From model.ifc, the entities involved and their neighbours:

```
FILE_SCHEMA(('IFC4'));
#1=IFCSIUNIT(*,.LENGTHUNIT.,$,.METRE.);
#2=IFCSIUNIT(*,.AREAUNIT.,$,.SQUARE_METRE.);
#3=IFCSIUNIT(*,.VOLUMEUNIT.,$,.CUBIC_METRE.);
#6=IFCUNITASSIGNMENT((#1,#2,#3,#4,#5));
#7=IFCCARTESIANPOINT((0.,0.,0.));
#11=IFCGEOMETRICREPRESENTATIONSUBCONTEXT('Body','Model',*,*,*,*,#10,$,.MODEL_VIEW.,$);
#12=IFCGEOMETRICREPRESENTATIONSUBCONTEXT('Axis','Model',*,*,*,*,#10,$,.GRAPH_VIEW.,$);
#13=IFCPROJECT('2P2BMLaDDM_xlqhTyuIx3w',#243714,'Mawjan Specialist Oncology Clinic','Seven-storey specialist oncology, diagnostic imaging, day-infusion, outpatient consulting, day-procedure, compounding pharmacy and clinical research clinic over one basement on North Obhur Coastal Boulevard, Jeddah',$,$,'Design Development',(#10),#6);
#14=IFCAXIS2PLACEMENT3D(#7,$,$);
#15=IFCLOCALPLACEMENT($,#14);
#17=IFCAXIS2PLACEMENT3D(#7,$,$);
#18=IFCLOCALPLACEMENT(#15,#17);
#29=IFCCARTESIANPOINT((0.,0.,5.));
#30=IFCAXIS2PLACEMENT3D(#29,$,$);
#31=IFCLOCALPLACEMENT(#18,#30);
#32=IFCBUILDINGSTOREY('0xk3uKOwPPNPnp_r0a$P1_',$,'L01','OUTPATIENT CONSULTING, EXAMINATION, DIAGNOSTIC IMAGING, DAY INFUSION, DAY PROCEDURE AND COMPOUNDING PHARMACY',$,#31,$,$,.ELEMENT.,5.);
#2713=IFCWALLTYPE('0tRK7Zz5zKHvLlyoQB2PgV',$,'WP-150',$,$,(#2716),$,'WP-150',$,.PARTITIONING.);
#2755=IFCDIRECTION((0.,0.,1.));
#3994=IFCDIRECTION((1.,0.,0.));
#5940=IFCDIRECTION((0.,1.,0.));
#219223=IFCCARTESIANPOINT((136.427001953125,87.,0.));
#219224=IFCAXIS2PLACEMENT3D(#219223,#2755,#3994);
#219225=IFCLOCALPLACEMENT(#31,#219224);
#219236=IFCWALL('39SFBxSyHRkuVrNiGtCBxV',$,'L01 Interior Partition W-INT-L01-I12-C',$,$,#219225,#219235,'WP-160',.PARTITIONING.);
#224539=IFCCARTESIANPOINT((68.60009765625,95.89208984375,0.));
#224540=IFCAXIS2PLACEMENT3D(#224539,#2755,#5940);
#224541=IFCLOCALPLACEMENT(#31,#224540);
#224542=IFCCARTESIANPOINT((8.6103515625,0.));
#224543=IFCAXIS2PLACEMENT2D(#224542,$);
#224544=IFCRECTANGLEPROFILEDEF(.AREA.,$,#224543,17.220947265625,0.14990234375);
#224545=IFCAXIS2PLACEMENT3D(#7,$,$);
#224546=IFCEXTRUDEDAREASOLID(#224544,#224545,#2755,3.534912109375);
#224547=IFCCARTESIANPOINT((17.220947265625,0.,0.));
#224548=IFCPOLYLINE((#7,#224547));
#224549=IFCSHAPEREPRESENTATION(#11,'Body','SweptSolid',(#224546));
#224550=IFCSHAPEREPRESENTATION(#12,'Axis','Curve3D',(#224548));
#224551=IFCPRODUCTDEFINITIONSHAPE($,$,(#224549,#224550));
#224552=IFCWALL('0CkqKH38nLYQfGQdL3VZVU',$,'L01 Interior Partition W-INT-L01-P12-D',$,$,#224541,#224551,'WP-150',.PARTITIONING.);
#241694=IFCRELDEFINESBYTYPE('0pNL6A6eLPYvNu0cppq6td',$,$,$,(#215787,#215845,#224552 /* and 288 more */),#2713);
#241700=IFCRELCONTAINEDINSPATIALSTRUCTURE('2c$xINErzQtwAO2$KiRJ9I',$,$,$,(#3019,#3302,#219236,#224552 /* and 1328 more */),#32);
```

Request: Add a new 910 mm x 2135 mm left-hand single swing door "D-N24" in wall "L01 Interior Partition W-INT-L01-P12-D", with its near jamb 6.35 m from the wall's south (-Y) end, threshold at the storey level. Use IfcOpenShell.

```python
import numpy as np
import ifcopenshell
import ifcopenshell.api.feature
import ifcopenshell.api.geometry
import ifcopenshell.api.root
import ifcopenshell.api.spatial
import ifcopenshell.geom
import ifcopenshell.util.element
import ifcopenshell.util.placement
import ifcopenshell.util.representation
import ifcopenshell.util.shape
import ifcopenshell.util.unit

model = ifcopenshell.open("model.ifc")
unit_scale = ifcopenshell.util.unit.calculate_unit_scale(model)
settings = ifcopenshell.geom.settings()


def volume(element):
    """Net volume in cubic metres, openings subtracted."""
    shape = ifcopenshell.geom.create_shape(settings, element)
    return ifcopenshell.util.shape.get_volume(shape.geometry)


wall = model.by_id(224552)
storey = ifcopenshell.util.element.get_container(wall, ifc_class="IfcBuildingStorey")
context = ifcopenshell.util.representation.get_context(model, "Model", "Body", "MODEL_VIEW")
before = volume(wall)

width, height, from_end, sill = 0.91, 2.135, 6.35, 0.0  # metres

# The wall runs along its own X axis, and the end named is its -X end.
wall_shape = ifcopenshell.geom.create_shape(settings, wall)
x, y, z = ifcopenshell.util.shape.get_vertices(wall_shape.geometry).T
start = x.min() + from_end
face, thickness = float(y.min()), float(y.max() - y.min())
wall_matrix = ifcopenshell.util.placement.get_local_placement(wall.ObjectPlacement)
level = ifcopenshell.util.placement.get_local_placement(storey.ObjectPlacement)[2, 3]


def in_wall(x, y):
    """Placement at x, y metres in the wall's axes, at sill height."""
    matrix = wall_matrix.copy()
    matrix[:, 3] = wall_matrix @ np.array([x / unit_scale, y / unit_scale, 0.0, 1.0])
    matrix[2, 3] = level + sill / unit_scale
    return matrix


# Opening: a box that overshoots both wall faces by 50 mm.
opening = ifcopenshell.api.root.create_entity(model, ifc_class="IfcOpeningElement", predefined_type="OPENING")
box = ifcopenshell.api.geometry.add_wall_representation(
    model, context=context, length=width, height=height, thickness=thickness + 0.1
)
ifcopenshell.api.geometry.assign_representation(model, product=opening, representation=box)
ifcopenshell.api.geometry.edit_object_placement(model, product=opening, matrix=in_wall(start, face - 0.05), is_si=False)
ifcopenshell.api.feature.add_feature(model, feature=opening, element=wall)

door = ifcopenshell.api.root.create_entity(model, ifc_class="IfcDoor", name="D-N24", predefined_type="DOOR")
door.OverallWidth, door.OverallHeight = width / unit_scale, height / unit_scale
door.OperationType = "SINGLE_SWING_LEFT"
body = ifcopenshell.api.geometry.add_door_representation(
    model,
    context=context,
    overall_width=door.OverallWidth,
    overall_height=door.OverallHeight,
    operation_type="SINGLE_SWING_LEFT",
    lining_properties={"LiningDepth": thickness / unit_scale, "ThresholdDepth": thickness / unit_scale},
)
ifcopenshell.api.geometry.assign_representation(model, product=door, representation=body)
ifcopenshell.api.spatial.assign_container(model, products=[door], relating_structure=storey)
ifcopenshell.api.feature.add_filling(model, opening=opening, element=door)

# The lining spans the wall, so the door starts at the wall face.
ifcopenshell.api.geometry.edit_object_placement(model, product=door, matrix=in_wall(start, face), is_si=False)

after = volume(wall)

print(f"wall volume {before:.3f} -> {after:.3f} m3")

model.write("model_edited.ifc")
```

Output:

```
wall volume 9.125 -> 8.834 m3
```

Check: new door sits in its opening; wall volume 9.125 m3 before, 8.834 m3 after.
